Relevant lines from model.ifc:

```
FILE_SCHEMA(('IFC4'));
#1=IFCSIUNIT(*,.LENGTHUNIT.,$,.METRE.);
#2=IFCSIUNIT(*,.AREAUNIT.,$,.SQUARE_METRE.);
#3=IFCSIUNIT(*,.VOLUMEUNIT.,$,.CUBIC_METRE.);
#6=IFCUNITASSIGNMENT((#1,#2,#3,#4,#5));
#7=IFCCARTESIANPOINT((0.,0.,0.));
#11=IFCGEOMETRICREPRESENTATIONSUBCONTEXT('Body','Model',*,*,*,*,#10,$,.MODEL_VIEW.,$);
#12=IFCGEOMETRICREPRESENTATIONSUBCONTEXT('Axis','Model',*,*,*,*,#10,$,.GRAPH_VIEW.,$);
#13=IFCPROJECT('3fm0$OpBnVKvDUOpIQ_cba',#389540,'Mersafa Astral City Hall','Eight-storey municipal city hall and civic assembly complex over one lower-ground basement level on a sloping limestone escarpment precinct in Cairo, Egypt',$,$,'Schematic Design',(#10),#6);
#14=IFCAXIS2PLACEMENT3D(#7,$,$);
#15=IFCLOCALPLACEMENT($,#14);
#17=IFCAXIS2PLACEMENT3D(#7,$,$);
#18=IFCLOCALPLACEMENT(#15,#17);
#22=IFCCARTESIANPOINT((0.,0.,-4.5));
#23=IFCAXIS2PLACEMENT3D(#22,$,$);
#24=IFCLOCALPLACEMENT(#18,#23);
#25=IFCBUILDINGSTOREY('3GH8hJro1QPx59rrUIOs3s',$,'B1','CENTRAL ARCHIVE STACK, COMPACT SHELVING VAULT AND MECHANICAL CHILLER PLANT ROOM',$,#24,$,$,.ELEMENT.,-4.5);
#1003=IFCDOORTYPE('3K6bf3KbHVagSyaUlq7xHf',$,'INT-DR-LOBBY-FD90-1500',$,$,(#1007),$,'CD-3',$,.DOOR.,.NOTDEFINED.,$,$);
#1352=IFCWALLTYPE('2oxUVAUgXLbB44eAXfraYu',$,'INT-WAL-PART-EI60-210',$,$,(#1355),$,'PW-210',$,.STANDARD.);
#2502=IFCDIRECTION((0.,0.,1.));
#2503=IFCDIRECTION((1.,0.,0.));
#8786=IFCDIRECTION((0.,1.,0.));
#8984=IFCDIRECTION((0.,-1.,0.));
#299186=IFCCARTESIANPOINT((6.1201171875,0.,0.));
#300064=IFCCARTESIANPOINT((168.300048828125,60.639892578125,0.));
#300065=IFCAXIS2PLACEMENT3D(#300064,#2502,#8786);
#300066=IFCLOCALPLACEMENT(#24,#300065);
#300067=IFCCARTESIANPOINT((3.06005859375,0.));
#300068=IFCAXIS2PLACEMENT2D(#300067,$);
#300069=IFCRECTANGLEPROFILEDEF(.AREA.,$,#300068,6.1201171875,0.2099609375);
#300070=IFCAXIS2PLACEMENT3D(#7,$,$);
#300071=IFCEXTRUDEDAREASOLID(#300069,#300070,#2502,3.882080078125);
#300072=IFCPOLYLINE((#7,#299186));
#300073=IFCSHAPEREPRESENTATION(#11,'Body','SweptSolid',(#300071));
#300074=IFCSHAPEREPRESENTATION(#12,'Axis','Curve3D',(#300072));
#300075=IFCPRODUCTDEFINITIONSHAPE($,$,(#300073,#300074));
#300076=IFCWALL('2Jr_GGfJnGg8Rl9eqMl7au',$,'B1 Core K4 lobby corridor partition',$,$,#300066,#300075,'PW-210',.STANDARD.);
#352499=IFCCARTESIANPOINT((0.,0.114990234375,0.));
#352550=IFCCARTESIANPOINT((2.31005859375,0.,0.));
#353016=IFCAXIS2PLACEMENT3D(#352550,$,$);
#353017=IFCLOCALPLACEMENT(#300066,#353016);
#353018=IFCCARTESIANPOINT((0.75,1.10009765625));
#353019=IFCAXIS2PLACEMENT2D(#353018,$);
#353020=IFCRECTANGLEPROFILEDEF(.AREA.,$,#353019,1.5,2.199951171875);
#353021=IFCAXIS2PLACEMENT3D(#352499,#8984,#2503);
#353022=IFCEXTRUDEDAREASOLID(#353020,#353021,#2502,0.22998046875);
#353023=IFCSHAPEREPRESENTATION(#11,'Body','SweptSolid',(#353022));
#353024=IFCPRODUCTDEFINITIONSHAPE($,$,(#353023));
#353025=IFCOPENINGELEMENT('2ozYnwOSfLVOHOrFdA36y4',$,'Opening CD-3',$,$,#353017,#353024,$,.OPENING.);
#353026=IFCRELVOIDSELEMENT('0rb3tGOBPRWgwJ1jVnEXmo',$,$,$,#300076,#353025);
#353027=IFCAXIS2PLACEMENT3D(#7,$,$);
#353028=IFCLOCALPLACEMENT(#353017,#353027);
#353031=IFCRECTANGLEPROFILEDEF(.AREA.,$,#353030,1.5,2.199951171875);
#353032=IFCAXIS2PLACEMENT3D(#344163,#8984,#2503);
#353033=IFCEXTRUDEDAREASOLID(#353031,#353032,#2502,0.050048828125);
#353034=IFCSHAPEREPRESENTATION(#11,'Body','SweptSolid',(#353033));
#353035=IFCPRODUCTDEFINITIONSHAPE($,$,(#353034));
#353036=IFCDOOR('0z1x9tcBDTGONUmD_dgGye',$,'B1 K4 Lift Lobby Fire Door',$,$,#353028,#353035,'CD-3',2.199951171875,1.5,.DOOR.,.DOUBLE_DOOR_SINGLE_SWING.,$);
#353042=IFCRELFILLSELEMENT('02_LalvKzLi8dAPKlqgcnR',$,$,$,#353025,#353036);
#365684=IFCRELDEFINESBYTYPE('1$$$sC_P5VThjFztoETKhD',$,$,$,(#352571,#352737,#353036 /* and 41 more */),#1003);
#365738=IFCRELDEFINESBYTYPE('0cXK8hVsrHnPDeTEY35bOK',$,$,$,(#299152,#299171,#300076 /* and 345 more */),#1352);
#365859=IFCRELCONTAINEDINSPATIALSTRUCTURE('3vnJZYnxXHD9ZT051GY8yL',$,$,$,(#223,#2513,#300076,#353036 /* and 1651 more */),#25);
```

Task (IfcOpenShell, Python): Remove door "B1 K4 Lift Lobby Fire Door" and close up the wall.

```python
import ifcopenshell
import ifcopenshell.api.feature
import ifcopenshell.api.root
import ifcopenshell.geom
import ifcopenshell.util.shape

model = ifcopenshell.open("model.ifc")
settings = ifcopenshell.geom.settings()


def volume(element):
    """Net volume in cubic metres, openings subtracted."""
    shape = ifcopenshell.geom.create_shape(settings, element)
    return ifcopenshell.util.shape.get_volume(shape.geometry)


door = model.by_guid("0z1x9tcBDTGONUmD_dgGye")
opening = door.FillsVoids[0].RelatingOpeningElement
wall = opening.VoidsElements[0].RelatingBuildingElement
before = volume(wall)

ifcopenshell.api.root.remove_product(model, product=door)
ifcopenshell.api.feature.remove_feature(model, feature=opening)

after = volume(wall)

print(f"wall volume {before:.3f} -> {after:.3f} m3")

model.write("model_updated.ifc")
```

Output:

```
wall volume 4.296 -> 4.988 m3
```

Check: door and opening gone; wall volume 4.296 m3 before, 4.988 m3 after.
